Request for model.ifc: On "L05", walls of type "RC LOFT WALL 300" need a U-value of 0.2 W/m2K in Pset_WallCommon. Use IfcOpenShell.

First a look at what the model holds.

```python
import ifcopenshell
import ifcopenshell.util.element

model = ifcopenshell.open("model.ifc")
print(model.schema)
storey = next(s for s in model.by_type("IfcBuildingStorey") if s.Name == "L05")
walls = [e for e in ifcopenshell.util.element.get_decomposition(storey) if e.is_a("IfcWall")]
seen = {}
for e in walls:
    element_type = ifcopenshell.util.element.get_type(e)
    key = (element_type.Name if element_type != e and element_type else None, ifcopenshell.util.element.get_pset(e, "Pset_WallCommon", "ThermalTransmittance"))
    seen[key] = seen.get(key, 0) + 1
for (name, value), count in sorted(seen.items(), key=str):
    print(count, "x", name, "|", value)
```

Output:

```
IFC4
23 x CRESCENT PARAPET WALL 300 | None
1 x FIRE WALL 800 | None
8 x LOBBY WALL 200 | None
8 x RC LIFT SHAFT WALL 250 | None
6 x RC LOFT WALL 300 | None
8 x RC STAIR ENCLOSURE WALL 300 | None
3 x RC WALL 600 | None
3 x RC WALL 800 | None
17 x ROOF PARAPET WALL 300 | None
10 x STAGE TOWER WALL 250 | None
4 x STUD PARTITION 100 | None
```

```python
import ifcopenshell
import ifcopenshell.api.pset
import ifcopenshell.util.element

model = ifcopenshell.open("model.ifc")

storey = next(s for s in model.by_type("IfcBuildingStorey") if s.Name == "L05")
walls = [e for e in ifcopenshell.util.element.get_decomposition(storey) if e.is_a("IfcWall")]

count = 0
for e in walls:
    element_type = ifcopenshell.util.element.get_type(e)
    if element_type in (None, e) or element_type.Name != "RC LOFT WALL 300":
        continue
    # add_pset returns the element's existing set when there is one.
    pset = ifcopenshell.api.pset.add_pset(model, product=e, name="Pset_WallCommon")
    ifcopenshell.api.pset.edit_pset(model, pset=pset, properties={"ThermalTransmittance": 0.2})
    count += 1

print(count, "walls updated")

model.write("model-out.ifc")
```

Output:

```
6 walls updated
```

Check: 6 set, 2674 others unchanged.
